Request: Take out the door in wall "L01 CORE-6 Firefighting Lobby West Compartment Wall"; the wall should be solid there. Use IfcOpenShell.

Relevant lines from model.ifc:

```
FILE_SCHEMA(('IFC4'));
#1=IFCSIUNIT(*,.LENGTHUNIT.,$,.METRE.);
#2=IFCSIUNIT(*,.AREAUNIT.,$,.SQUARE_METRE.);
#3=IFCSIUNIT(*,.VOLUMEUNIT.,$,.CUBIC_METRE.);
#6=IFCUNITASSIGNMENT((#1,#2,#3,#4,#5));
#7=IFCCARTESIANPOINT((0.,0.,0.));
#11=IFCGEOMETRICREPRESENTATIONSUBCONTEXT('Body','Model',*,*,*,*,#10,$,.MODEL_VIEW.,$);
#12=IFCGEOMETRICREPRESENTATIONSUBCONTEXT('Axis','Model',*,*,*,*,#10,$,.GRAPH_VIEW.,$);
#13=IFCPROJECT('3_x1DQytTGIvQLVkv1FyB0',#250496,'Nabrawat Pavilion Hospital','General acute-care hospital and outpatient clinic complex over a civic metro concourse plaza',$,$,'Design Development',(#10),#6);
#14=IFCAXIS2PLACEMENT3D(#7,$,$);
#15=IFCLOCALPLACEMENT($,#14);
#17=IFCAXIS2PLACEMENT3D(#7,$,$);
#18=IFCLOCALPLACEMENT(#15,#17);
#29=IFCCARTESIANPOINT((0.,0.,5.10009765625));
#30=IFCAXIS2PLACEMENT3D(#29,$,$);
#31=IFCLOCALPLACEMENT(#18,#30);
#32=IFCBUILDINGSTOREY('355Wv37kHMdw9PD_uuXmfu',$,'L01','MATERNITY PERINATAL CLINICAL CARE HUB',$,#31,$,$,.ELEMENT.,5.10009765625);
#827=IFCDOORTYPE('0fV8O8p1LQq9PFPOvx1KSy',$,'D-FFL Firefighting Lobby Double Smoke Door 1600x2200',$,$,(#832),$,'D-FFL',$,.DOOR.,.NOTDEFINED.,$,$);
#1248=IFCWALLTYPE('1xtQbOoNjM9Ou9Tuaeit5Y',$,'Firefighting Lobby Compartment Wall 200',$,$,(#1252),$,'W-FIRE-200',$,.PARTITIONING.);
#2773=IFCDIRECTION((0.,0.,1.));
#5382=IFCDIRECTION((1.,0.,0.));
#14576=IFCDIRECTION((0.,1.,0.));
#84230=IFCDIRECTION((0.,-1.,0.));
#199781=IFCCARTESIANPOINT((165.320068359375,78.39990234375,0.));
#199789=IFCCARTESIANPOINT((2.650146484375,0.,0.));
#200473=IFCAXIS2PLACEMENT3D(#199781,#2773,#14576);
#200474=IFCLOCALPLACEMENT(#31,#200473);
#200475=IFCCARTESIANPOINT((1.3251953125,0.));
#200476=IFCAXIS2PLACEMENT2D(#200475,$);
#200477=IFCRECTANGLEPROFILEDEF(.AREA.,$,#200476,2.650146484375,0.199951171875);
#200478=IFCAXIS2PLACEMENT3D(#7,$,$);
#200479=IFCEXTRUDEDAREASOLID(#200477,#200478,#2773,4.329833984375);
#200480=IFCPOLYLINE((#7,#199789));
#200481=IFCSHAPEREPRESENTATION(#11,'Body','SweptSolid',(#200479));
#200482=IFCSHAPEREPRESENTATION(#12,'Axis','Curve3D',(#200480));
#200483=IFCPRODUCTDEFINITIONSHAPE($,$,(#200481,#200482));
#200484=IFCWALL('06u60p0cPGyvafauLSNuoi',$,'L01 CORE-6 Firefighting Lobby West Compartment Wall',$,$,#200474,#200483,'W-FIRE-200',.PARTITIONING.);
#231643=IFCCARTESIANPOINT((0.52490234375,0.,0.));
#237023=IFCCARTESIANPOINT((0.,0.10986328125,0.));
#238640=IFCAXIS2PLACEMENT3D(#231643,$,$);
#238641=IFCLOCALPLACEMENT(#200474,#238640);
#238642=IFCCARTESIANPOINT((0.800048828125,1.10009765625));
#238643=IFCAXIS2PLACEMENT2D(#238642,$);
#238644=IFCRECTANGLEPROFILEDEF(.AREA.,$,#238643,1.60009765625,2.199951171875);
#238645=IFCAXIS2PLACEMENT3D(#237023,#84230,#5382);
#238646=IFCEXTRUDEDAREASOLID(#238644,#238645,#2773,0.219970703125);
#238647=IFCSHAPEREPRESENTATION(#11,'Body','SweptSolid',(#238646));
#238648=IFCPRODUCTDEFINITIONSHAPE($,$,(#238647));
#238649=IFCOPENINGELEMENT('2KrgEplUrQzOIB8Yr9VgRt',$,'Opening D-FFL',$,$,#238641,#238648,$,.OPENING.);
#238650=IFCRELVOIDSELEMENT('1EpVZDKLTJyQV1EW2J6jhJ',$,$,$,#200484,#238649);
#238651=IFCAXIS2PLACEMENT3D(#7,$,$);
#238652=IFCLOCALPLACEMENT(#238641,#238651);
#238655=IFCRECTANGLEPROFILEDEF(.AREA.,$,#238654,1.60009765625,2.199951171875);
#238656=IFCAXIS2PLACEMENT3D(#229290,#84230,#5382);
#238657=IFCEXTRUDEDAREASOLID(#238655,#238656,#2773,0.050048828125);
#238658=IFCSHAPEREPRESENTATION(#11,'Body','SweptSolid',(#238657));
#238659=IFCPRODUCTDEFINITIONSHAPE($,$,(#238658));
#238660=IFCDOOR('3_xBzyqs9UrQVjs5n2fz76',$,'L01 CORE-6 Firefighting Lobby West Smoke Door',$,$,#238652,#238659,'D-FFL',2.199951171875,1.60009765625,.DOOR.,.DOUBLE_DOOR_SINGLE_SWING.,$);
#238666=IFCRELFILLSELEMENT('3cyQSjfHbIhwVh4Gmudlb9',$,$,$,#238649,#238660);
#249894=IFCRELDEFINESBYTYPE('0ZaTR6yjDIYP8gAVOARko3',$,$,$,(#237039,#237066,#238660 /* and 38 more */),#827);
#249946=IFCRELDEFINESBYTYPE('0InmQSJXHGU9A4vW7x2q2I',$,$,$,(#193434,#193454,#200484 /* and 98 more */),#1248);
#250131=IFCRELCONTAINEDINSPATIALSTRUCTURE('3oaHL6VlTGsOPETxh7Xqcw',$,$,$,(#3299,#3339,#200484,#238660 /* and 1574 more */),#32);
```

```python
import ifcopenshell
import ifcopenshell.api.feature
import ifcopenshell.api.root
import ifcopenshell.geom
import ifcopenshell.util.shape

model = ifcopenshell.open("model.ifc")
settings = ifcopenshell.geom.settings()


def volume(element):
    """Net volume in cubic metres, openings subtracted."""
    shape = ifcopenshell.geom.create_shape(settings, element)
    return ifcopenshell.util.shape.get_volume(shape.geometry)


door = model.by_guid("3_xBzyqs9UrQVjs5n2fz76")
opening = door.FillsVoids[0].RelatingOpeningElement
wall = opening.VoidsElements[0].RelatingBuildingElement
before = volume(wall)

ifcopenshell.api.root.remove_product(model, product=door)
ifcopenshell.api.feature.remove_feature(model, feature=opening)

after = volume(wall)

print(f"wall volume {before:.3f} -> {after:.3f} m3")

model.write("model_edited.ifc")
```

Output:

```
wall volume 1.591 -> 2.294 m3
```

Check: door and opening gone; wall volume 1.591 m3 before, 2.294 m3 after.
